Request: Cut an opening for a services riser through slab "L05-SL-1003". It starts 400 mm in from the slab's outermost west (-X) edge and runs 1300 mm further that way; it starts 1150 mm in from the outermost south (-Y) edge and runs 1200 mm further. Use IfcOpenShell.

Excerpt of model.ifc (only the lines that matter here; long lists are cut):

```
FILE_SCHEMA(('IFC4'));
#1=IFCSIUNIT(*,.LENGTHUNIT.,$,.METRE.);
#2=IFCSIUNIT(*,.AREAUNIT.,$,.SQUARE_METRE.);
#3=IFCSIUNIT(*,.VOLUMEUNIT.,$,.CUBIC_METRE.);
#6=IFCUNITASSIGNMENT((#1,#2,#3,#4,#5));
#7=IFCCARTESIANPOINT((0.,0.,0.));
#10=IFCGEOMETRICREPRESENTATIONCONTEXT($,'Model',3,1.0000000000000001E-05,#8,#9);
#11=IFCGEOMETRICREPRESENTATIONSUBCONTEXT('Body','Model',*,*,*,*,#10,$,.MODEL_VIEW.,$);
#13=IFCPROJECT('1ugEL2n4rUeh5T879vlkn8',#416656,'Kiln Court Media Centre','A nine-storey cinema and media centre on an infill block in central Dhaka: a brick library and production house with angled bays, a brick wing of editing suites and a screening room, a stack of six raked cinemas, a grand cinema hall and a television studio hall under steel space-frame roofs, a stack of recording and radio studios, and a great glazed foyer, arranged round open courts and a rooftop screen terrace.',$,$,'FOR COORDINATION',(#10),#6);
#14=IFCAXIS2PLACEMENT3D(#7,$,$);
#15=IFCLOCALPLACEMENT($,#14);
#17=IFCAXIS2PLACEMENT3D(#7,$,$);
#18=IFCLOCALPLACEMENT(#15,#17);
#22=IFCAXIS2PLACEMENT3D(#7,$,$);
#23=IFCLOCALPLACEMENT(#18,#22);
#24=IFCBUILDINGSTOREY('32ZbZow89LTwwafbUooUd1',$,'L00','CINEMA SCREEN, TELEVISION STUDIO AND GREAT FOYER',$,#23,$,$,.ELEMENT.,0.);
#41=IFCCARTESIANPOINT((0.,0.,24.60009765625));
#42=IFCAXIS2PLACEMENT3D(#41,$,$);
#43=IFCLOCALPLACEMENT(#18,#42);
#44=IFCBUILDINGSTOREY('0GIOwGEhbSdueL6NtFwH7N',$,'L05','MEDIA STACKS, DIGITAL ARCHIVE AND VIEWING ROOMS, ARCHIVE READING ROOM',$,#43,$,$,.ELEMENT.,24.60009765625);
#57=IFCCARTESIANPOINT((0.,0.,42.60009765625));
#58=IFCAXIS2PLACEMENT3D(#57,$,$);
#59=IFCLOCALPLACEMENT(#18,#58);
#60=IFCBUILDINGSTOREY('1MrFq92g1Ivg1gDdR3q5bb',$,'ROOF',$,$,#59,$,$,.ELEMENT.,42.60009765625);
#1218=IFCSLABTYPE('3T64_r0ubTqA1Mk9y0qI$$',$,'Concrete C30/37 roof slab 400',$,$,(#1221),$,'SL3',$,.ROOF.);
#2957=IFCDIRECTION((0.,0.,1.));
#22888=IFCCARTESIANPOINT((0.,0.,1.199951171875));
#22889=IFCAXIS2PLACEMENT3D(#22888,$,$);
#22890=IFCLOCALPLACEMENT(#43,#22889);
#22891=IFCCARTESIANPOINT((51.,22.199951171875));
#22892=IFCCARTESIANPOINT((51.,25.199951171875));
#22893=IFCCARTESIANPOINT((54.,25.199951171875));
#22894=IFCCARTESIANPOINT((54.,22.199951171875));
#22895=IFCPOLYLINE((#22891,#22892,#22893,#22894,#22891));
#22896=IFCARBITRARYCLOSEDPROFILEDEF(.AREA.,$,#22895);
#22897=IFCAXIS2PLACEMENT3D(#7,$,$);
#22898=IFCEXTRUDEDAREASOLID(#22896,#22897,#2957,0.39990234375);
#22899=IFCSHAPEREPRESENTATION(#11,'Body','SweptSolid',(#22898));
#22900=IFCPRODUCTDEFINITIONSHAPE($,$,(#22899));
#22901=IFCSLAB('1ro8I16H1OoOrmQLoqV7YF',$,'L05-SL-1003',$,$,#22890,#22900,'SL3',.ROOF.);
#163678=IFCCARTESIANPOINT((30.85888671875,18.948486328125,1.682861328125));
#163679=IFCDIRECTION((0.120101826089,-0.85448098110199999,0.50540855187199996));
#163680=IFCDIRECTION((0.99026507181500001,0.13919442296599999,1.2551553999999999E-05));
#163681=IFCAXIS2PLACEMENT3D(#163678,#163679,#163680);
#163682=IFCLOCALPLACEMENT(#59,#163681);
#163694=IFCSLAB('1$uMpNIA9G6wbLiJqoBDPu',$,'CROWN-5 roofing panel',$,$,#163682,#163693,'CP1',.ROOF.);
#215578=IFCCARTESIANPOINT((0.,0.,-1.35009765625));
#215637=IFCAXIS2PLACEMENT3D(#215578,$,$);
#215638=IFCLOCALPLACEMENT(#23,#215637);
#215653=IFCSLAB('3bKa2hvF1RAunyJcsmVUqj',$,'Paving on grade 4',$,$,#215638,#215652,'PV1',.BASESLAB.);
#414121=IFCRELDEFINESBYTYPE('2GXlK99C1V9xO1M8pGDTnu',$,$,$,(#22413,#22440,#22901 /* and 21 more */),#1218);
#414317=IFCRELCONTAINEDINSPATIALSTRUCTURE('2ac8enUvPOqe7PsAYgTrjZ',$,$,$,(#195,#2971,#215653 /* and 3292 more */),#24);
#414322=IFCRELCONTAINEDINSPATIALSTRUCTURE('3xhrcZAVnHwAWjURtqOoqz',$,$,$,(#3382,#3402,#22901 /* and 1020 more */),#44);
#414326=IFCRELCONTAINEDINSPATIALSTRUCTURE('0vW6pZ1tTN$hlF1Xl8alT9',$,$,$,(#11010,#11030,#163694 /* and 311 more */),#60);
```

```python
import numpy as np
import ifcopenshell
import ifcopenshell.api.feature
import ifcopenshell.api.geometry
import ifcopenshell.api.root
import ifcopenshell.geom
import ifcopenshell.util.placement
import ifcopenshell.util.representation
import ifcopenshell.util.shape
import ifcopenshell.util.unit

model = ifcopenshell.open("model.ifc")
unit_scale = ifcopenshell.util.unit.calculate_unit_scale(model)
settings = ifcopenshell.geom.settings()


def volume(element):
    """Net volume in cubic metres, openings subtracted."""
    shape = ifcopenshell.geom.create_shape(settings, element)
    return ifcopenshell.util.shape.get_volume(shape.geometry)


slab = model.by_guid("1ro8I16H1OoOrmQLoqV7YF")
before = volume(slab)

# Extent in the slab's own axes, in metres. The edges named are its -X and -Y sides.
slab_shape = ifcopenshell.geom.create_shape(settings, slab)
vertices = ifcopenshell.util.shape.get_vertices(slab_shape.geometry)
x_min, y_min, bottom = vertices.min(axis=0)
top = vertices[:, 2].max()

opening = ifcopenshell.api.root.create_entity(model, ifc_class="IfcOpeningElement", name="Services riser opening", predefined_type="OPENING")
context = ifcopenshell.util.representation.get_context(model, "Model", "Body", "MODEL_VIEW")
width, depth = 1.3, 1.2
outline = [(0.0, 0.0), (width, 0.0), (width, depth), (0.0, depth), (0.0, 0.0)]
# Overshoot both faces by 50 mm so the cut is clean.
shape = ifcopenshell.api.geometry.add_slab_representation(
    model, context=context, depth=top - bottom + 0.1, polyline=outline
)
ifcopenshell.api.geometry.assign_representation(model, product=opening, representation=shape)

matrix = ifcopenshell.util.placement.get_local_placement(slab.ObjectPlacement)
matrix[:, 3] = matrix @ np.append(np.array([x_min + 0.4, y_min + 1.15, bottom - 0.05]) / unit_scale, 1.0)
ifcopenshell.api.geometry.edit_object_placement(model, product=opening, matrix=matrix, is_si=False)
ifcopenshell.api.feature.add_feature(model, feature=opening, element=slab)

after = volume(slab)

print(f"slab volume {before:.3f} -> {after:.3f} m3")

model.write("model_updated.ifc")
```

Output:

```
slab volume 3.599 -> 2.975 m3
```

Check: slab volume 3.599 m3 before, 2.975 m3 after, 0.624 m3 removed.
